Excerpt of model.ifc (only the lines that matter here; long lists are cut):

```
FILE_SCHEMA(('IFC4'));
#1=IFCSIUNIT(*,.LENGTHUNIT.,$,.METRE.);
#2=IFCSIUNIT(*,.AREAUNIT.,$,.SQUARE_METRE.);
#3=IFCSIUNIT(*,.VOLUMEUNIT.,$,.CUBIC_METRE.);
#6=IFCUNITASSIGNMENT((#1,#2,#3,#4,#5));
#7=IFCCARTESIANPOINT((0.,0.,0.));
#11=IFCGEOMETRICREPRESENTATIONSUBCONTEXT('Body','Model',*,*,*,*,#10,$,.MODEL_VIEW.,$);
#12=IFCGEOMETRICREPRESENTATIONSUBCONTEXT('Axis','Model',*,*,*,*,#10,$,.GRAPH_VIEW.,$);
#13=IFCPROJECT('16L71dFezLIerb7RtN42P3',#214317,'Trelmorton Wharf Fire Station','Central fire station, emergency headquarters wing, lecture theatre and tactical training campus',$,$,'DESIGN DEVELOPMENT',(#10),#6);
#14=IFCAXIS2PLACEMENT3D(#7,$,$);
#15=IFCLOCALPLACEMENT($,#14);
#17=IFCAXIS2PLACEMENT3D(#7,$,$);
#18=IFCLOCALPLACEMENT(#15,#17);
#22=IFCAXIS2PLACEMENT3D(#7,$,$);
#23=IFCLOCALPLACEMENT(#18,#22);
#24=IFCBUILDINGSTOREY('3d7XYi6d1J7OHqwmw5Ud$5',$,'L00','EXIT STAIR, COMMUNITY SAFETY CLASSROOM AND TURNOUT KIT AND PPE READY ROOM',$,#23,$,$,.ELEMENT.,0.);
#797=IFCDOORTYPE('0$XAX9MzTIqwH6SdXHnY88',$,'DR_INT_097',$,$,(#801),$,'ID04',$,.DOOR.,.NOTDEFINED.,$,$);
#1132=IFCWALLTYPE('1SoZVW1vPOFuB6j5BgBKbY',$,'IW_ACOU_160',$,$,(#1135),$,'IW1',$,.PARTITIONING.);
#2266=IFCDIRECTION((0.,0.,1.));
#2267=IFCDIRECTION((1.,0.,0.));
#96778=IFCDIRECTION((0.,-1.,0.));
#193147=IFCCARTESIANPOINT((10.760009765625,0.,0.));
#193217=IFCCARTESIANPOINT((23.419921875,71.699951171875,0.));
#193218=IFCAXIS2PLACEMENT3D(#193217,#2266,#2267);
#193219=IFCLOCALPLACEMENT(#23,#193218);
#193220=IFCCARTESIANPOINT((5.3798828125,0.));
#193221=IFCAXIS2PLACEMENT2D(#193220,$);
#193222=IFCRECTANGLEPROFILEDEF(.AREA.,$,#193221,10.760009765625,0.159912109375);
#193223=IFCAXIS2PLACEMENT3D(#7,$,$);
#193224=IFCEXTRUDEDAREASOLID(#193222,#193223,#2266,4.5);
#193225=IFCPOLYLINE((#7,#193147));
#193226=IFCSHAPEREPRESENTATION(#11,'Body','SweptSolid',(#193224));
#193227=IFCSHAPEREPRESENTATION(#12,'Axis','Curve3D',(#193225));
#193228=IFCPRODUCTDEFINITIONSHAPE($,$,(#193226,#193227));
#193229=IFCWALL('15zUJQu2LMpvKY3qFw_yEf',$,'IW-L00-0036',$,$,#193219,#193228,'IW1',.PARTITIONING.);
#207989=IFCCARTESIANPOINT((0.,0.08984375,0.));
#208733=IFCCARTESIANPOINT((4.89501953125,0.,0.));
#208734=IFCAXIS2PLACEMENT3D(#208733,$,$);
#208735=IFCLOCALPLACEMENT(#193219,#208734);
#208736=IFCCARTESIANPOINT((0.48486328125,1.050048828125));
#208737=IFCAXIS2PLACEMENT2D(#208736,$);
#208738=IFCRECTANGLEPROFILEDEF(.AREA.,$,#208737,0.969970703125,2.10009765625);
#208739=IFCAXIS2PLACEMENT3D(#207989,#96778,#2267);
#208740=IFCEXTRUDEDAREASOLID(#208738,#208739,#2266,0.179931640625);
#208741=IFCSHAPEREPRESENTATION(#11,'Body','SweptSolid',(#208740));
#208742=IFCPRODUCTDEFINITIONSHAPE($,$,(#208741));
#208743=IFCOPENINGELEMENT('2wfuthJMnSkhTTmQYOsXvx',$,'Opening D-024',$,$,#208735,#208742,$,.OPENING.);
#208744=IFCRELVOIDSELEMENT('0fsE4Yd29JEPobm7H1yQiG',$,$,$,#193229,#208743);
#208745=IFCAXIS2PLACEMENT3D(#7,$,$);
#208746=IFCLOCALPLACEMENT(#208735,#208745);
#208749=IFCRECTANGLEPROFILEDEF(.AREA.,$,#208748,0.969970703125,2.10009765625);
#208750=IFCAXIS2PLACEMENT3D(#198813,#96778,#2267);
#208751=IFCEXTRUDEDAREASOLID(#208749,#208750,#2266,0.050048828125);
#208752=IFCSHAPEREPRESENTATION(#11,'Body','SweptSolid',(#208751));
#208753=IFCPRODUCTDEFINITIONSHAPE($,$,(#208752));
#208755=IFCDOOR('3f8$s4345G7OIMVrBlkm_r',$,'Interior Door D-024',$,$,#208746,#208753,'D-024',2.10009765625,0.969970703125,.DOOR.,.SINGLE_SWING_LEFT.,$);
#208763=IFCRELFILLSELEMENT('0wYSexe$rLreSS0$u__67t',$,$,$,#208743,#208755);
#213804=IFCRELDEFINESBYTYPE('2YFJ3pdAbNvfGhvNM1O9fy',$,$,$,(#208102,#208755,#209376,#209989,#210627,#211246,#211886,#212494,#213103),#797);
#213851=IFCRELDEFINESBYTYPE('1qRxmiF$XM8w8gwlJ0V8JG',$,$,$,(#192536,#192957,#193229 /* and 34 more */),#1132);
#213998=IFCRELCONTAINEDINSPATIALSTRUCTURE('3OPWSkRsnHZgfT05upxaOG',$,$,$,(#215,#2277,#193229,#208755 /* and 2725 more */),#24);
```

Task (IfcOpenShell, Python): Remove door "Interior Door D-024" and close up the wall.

```python
import ifcopenshell
import ifcopenshell.api.feature
import ifcopenshell.api.root
import ifcopenshell.geom
import ifcopenshell.util.shape

model = ifcopenshell.open("model.ifc")
settings = ifcopenshell.geom.settings()


def volume(element):
    """Net volume in cubic metres, openings subtracted."""
    shape = ifcopenshell.geom.create_shape(settings, element)
    return ifcopenshell.util.shape.get_volume(shape.geometry)


door = model.by_guid("3f8$s4345G7OIMVrBlkm_r")
opening = door.FillsVoids[0].RelatingOpeningElement
wall = opening.VoidsElements[0].RelatingBuildingElement
before = volume(wall)

ifcopenshell.api.root.remove_product(model, product=door)
ifcopenshell.api.feature.remove_feature(model, feature=opening)

after = volume(wall)

print(f"wall volume {before:.3f} -> {after:.3f} m3")

model.write("model_v2.ifc")
```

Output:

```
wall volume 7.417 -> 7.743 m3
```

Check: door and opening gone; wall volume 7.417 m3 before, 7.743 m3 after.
